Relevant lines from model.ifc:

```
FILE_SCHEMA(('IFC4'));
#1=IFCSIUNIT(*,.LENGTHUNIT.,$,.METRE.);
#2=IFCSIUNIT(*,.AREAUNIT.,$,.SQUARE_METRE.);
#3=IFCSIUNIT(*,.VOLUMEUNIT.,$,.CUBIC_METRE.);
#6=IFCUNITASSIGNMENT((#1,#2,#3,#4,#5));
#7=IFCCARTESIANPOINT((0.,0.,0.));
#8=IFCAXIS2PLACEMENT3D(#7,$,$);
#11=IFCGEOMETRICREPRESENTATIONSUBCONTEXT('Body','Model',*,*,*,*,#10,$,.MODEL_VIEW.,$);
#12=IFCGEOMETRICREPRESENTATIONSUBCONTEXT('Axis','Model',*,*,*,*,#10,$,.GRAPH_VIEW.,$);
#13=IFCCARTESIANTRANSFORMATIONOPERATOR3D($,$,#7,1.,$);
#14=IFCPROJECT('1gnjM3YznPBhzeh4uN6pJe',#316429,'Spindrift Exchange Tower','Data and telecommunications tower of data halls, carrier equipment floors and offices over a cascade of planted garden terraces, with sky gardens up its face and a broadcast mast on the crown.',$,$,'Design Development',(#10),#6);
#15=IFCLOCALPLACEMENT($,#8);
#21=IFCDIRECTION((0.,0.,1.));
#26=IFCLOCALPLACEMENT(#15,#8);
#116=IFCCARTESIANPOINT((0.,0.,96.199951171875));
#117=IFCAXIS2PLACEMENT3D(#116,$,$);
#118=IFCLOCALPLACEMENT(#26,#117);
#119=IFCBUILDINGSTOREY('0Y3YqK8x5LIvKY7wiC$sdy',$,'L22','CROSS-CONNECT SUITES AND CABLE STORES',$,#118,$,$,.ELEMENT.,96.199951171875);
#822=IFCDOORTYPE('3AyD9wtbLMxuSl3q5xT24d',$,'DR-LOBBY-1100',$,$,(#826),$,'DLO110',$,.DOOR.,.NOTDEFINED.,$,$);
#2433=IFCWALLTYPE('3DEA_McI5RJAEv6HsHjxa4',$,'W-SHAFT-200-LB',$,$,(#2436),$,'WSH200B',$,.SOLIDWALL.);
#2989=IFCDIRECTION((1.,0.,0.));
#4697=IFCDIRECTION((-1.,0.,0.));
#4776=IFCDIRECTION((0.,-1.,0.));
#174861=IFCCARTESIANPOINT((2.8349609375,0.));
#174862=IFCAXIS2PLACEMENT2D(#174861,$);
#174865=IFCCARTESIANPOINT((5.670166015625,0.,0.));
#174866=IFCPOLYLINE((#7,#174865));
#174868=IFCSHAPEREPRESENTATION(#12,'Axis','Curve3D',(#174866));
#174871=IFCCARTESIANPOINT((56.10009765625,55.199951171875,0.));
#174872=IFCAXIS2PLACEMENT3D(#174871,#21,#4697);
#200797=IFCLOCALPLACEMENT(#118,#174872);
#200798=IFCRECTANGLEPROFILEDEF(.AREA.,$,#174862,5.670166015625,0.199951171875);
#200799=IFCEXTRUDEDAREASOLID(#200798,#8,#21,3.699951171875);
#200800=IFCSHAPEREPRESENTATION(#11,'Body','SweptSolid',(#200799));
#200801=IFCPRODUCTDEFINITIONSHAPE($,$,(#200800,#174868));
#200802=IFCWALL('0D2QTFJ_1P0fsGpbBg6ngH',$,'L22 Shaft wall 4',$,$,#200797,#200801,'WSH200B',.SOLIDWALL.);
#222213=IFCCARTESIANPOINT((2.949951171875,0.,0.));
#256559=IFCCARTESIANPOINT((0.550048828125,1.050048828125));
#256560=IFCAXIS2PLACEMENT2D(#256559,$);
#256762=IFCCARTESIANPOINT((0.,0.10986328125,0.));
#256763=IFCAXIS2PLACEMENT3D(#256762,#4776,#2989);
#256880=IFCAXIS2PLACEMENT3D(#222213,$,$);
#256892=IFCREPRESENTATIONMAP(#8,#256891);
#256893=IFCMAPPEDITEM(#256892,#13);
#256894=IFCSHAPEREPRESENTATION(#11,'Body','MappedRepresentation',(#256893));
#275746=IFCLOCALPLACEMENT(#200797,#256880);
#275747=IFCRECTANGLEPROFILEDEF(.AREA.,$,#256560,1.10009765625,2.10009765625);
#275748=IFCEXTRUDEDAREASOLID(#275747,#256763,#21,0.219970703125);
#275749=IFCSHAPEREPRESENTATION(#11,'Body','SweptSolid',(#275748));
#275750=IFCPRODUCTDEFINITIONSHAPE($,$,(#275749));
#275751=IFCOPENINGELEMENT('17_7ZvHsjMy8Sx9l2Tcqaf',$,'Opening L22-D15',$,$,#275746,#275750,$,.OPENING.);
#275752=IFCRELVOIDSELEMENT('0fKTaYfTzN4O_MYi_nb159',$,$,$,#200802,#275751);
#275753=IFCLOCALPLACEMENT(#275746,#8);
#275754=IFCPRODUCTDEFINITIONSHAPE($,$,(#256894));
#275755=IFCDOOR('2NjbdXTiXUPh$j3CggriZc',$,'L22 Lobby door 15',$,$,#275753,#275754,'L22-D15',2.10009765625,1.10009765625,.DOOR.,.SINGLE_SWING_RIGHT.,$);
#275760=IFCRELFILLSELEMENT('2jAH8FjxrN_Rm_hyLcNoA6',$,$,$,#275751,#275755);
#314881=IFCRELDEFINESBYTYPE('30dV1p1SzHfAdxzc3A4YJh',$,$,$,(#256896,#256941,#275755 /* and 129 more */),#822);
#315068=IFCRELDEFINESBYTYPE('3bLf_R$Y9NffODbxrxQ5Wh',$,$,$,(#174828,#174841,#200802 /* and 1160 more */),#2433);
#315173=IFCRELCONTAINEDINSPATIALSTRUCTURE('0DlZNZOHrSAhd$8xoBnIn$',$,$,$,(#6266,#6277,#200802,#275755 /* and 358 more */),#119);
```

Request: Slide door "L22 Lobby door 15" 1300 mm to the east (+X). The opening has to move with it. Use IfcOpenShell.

```python
import ifcopenshell
import ifcopenshell.api.geometry
import ifcopenshell.util.placement
import ifcopenshell.util.unit

model = ifcopenshell.open("model.ifc")
unit_scale = ifcopenshell.util.unit.calculate_unit_scale(model)

door = model.by_id(275755)
opening = door.FillsVoids[0].RelatingOpeningElement
wall = opening.VoidsElements[0].RelatingBuildingElement

wall_matrix = ifcopenshell.util.placement.get_local_placement(wall.ObjectPlacement)
shift = wall_matrix[:3, 0] * -1.3 / unit_scale
before = ifcopenshell.util.placement.get_local_placement(door.ObjectPlacement)[:3, 3].copy()

# The door is placed relative to its opening, so it follows when the opening moves.
matrix = ifcopenshell.util.placement.get_local_placement(opening.ObjectPlacement)
matrix[:3, 3] += shift
ifcopenshell.api.geometry.edit_object_placement(
    model, product=opening, matrix=matrix, is_si=False, should_transform_children=True
)

after = ifcopenshell.util.placement.get_local_placement(door.ObjectPlacement)[:3, 3]
print("door moved by", (after - before).round(3) + 0.0)

model.write("model_rev.ifc")
```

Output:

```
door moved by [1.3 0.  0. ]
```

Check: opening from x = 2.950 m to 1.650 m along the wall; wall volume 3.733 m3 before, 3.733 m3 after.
